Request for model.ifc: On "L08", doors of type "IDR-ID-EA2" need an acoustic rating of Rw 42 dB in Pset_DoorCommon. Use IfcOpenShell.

First a look at what the model holds.

```python
import ifcopenshell
import ifcopenshell.util.element

model = ifcopenshell.open("model.ifc")
print(model.schema)
storey = next(s for s in model.by_type("IfcBuildingStorey") if s.Name == "L08")
doors = [e for e in ifcopenshell.util.element.get_decomposition(storey) if e.is_a("IfcDoor")]
seen = {}
for e in doors:
    element_type = ifcopenshell.util.element.get_type(e)
    key = (element_type.Name if element_type != e and element_type else None, ifcopenshell.util.element.get_pset(e, "Pset_DoorCommon", "AcousticRating"))
    seen[key] = seen.get(key, 0) + 1
for (name, value), count in sorted(seen.items(), key=str):
    print(count, "x", name, "|", value)
```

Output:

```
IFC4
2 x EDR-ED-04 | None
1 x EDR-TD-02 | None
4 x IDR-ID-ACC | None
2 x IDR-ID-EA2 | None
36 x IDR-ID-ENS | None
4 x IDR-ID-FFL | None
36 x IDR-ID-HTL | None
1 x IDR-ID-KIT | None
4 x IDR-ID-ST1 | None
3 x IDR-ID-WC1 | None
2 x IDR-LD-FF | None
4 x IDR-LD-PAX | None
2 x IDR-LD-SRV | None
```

```python
import ifcopenshell
import ifcopenshell.api.pset
import ifcopenshell.util.element

model = ifcopenshell.open("model.ifc")

storey = next(s for s in model.by_type("IfcBuildingStorey") if s.Name == "L08")
doors = [e for e in ifcopenshell.util.element.get_decomposition(storey) if e.is_a("IfcDoor")]

count = 0
for e in doors:
    element_type = ifcopenshell.util.element.get_type(e)
    if element_type in (None, e) or element_type.Name != "IDR-ID-EA2":
        continue
    # add_pset returns the element's existing set when there is one.
    pset = ifcopenshell.api.pset.add_pset(model, product=e, name="Pset_DoorCommon")
    ifcopenshell.api.pset.edit_pset(model, pset=pset, properties={"AcousticRating": "Rw 42 dB"})
    count += 1

print(count, "doors updated")

model.write("model-out.ifc")
```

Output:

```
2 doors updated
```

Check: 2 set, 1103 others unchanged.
